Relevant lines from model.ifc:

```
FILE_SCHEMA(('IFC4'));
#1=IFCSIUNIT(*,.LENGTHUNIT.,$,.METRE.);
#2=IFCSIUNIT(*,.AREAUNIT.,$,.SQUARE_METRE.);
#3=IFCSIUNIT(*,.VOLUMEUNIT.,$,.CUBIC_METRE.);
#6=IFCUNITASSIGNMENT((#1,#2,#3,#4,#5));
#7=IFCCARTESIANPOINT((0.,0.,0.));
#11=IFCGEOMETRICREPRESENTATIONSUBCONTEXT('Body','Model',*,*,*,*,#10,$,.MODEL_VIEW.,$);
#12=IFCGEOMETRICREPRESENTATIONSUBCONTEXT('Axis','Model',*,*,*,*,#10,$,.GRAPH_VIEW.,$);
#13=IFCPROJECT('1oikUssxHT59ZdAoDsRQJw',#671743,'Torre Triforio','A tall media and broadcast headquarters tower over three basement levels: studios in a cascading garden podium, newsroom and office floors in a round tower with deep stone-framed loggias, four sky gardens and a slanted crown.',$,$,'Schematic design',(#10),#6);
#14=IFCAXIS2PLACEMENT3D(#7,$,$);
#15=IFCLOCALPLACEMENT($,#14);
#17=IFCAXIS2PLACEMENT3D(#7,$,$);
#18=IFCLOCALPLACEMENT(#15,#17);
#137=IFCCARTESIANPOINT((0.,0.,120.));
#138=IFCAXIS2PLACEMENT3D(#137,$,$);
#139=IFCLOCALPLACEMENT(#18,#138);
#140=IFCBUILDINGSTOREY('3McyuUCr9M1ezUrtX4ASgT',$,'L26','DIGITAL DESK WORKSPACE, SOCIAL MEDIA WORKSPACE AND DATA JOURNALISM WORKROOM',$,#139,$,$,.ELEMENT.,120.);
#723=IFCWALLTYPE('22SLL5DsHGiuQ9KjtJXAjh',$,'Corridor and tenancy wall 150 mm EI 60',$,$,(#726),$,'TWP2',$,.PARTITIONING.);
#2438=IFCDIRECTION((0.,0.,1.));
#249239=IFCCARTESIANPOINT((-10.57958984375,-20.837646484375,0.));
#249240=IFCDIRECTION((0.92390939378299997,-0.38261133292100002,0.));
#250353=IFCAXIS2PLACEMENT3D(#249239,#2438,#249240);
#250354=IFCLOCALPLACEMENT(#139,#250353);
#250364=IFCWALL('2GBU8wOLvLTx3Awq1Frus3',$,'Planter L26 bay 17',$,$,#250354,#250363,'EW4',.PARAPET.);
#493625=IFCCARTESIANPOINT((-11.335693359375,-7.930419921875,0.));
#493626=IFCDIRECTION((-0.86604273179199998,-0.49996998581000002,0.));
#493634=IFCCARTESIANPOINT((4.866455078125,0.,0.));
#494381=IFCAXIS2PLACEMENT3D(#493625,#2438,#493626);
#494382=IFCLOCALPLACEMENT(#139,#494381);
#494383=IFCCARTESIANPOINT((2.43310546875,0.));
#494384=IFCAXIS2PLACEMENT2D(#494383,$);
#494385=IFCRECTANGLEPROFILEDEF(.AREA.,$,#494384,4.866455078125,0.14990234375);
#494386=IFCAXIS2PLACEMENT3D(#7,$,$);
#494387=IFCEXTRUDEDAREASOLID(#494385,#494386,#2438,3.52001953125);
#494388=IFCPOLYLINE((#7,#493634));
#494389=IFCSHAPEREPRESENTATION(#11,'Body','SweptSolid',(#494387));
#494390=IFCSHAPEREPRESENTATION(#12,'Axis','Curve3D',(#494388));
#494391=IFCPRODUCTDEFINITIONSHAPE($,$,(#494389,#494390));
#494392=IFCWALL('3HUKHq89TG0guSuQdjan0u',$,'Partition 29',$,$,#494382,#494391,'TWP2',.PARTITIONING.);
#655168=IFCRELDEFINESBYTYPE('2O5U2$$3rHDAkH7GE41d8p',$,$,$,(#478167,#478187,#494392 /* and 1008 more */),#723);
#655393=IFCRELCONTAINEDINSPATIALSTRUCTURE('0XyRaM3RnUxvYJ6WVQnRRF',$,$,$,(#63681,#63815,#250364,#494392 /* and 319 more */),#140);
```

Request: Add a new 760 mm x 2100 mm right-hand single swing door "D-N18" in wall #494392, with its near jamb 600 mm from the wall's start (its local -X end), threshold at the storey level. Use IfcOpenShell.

```python
import numpy as np
import ifcopenshell
import ifcopenshell.api.feature
import ifcopenshell.api.geometry
import ifcopenshell.api.root
import ifcopenshell.api.spatial
import ifcopenshell.geom
import ifcopenshell.util.element
import ifcopenshell.util.placement
import ifcopenshell.util.representation
import ifcopenshell.util.shape
import ifcopenshell.util.unit

model = ifcopenshell.open("model.ifc")
unit_scale = ifcopenshell.util.unit.calculate_unit_scale(model)
settings = ifcopenshell.geom.settings()


def volume(element):
    """Net volume in cubic metres, openings subtracted."""
    shape = ifcopenshell.geom.create_shape(settings, element)
    return ifcopenshell.util.shape.get_volume(shape.geometry)


wall = model.by_guid("3HUKHq89TG0guSuQdjan0u")
storey = ifcopenshell.util.element.get_container(wall, ifc_class="IfcBuildingStorey")
context = ifcopenshell.util.representation.get_context(model, "Model", "Body", "MODEL_VIEW")
before = volume(wall)

width, height, from_end, sill = 0.76, 2.1, 0.6, 0.0  # metres

# The wall runs along its own X axis, and the end named is its -X end.
wall_shape = ifcopenshell.geom.create_shape(settings, wall)
x, y, z = ifcopenshell.util.shape.get_vertices(wall_shape.geometry).T
start = x.min() + from_end
face, thickness = float(y.min()), float(y.max() - y.min())
wall_matrix = ifcopenshell.util.placement.get_local_placement(wall.ObjectPlacement)
level = ifcopenshell.util.placement.get_local_placement(storey.ObjectPlacement)[2, 3]


def in_wall(x, y):
    """Placement at x, y metres in the wall's axes, at sill height."""
    matrix = wall_matrix.copy()
    matrix[:, 3] = wall_matrix @ np.array([x / unit_scale, y / unit_scale, 0.0, 1.0])
    matrix[2, 3] = level + sill / unit_scale
    return matrix


# Opening: a box that overshoots both wall faces by 50 mm.
opening = ifcopenshell.api.root.create_entity(model, ifc_class="IfcOpeningElement", predefined_type="OPENING")
box = ifcopenshell.api.geometry.add_wall_representation(
    model, context=context, length=width, height=height, thickness=thickness + 0.1
)
ifcopenshell.api.geometry.assign_representation(model, product=opening, representation=box)
ifcopenshell.api.geometry.edit_object_placement(model, product=opening, matrix=in_wall(start, face - 0.05), is_si=False)
ifcopenshell.api.feature.add_feature(model, feature=opening, element=wall)

door = ifcopenshell.api.root.create_entity(model, ifc_class="IfcDoor", name="D-N18", predefined_type="DOOR")
door.OverallWidth, door.OverallHeight = width / unit_scale, height / unit_scale
door.OperationType = "SINGLE_SWING_RIGHT"
body = ifcopenshell.api.geometry.add_door_representation(
    model,
    context=context,
    overall_width=door.OverallWidth,
    overall_height=door.OverallHeight,
    operation_type="SINGLE_SWING_RIGHT",
    lining_properties={"LiningDepth": thickness / unit_scale, "ThresholdDepth": thickness / unit_scale},
)
ifcopenshell.api.geometry.assign_representation(model, product=door, representation=body)
ifcopenshell.api.spatial.assign_container(model, products=[door], relating_structure=storey)
ifcopenshell.api.feature.add_filling(model, opening=opening, element=door)

# The lining spans the wall, so the door starts at the wall face.
ifcopenshell.api.geometry.edit_object_placement(model, product=door, matrix=in_wall(start, face), is_si=False)

after = volume(wall)

print(f"wall volume {before:.3f} -> {after:.3f} m3")

model.write("model_updated.ifc")
```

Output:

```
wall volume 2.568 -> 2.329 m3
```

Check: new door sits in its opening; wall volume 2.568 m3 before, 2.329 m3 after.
